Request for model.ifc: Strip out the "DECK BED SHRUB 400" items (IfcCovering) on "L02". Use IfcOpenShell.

First a look at what the model holds.

```python
import ifcopenshell
import ifcopenshell.util.element

model = ifcopenshell.open("model.ifc")
print(model.schema)
storey = next(s for s in model.by_type("IfcBuildingStorey") if s.Name == "L02")
coverings = [e for e in ifcopenshell.util.element.get_decomposition(storey) if e.is_a("IfcCovering")]
seen = {}
for e in coverings:
    element_type = ifcopenshell.util.element.get_type(e)
    name = element_type.Name if element_type not in (None, e) else None
    seen[name] = seen.get(name, 0) + 1
for name, count in sorted(seen.items(), key=str):
    print(count, "x", name)
```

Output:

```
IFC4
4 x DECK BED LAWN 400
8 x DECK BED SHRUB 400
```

```python
import ifcopenshell
import ifcopenshell.api.root
import ifcopenshell.util.element

model = ifcopenshell.open("model.ifc")

storey = next(s for s in model.by_type("IfcBuildingStorey") if s.Name == "L02")
coverings = [e for e in ifcopenshell.util.element.get_decomposition(storey) if e.is_a("IfcCovering")]
targets = [e for e in coverings if (t := ifcopenshell.util.element.get_type(e)) not in (None, e) and t.Name == "DECK BED SHRUB 400"]

for e in targets:
    ifcopenshell.api.root.remove_product(model, product=e)
print(len(targets), "removed")

model.write("model_edited.ifc")
```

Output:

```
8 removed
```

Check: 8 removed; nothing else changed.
